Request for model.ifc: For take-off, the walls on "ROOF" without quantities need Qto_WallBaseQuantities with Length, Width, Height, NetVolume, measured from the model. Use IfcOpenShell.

First a look at what the model holds.

```python
import ifcopenshell
import ifcopenshell.util.element
import ifcopenshell.util.unit

model = ifcopenshell.open("model.ifc")
print(model.schema)
for unit_type in ("LENGTHUNIT", "AREAUNIT", "VOLUMEUNIT"):
    print(unit_type, ifcopenshell.util.unit.calculate_unit_scale(model, unit_type))
storey = next(s for s in model.by_type("IfcBuildingStorey") if s.Name == "ROOF")
walls = [e for e in ifcopenshell.util.element.get_decomposition(storey) if e.is_a("IfcWall")]
for e in sorted(walls, key=lambda e: e.id()):
    print(e.id(), e.is_a(), e.Name, list(ifcopenshell.util.element.get_psets(e, qtos_only=True)), sep=" | ")
```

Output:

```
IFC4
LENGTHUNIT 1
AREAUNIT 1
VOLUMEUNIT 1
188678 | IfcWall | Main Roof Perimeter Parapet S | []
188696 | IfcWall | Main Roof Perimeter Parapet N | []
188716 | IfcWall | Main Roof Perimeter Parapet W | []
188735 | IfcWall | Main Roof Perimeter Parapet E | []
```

```python
import ifcopenshell
import ifcopenshell.api.pset
import ifcopenshell.geom
import ifcopenshell.util.element
import ifcopenshell.util.shape
import ifcopenshell.util.unit

model = ifcopenshell.open("model.ifc")
unit_scale = ifcopenshell.util.unit.calculate_unit_scale(model)
volume_scale = ifcopenshell.util.unit.calculate_unit_scale(model, "VOLUMEUNIT")
settings = ifcopenshell.geom.settings()

storey = next(s for s in model.by_type("IfcBuildingStorey") if s.Name == "ROOF")
walls = [e for e in ifcopenshell.util.element.get_decomposition(storey) if e.is_a("IfcWall")]

for e in sorted(walls, key=lambda e: e.id()):
    if ifcopenshell.util.element.get_psets(e, qtos_only=True, should_inherit=False):
        continue
    # Geometry comes back in metres, in the element's own axes.
    shape = ifcopenshell.geom.create_shape(settings, e)
    values = {
        "Length": ifcopenshell.util.shape.get_x(shape.geometry) / unit_scale,
        "Width": ifcopenshell.util.shape.get_y(shape.geometry) / unit_scale,
        "Height": ifcopenshell.util.shape.get_z(shape.geometry) / unit_scale,
        "NetVolume": ifcopenshell.util.shape.get_volume(shape.geometry) / volume_scale,
    }
    qto = ifcopenshell.api.pset.add_qto(model, product=e, name="Qto_WallBaseQuantities")
    ifcopenshell.api.pset.edit_qto(model, qto=qto, properties=values)
    print(e.id(), {k: round(v, 3) for k, v in values.items()})

model.write("model_edited.ifc")
```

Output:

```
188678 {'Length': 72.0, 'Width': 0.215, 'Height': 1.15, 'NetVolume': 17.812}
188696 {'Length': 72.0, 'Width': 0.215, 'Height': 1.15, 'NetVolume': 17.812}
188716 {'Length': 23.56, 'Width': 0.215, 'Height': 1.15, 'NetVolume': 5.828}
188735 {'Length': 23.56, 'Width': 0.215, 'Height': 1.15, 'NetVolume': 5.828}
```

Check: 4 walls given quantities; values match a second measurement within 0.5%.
